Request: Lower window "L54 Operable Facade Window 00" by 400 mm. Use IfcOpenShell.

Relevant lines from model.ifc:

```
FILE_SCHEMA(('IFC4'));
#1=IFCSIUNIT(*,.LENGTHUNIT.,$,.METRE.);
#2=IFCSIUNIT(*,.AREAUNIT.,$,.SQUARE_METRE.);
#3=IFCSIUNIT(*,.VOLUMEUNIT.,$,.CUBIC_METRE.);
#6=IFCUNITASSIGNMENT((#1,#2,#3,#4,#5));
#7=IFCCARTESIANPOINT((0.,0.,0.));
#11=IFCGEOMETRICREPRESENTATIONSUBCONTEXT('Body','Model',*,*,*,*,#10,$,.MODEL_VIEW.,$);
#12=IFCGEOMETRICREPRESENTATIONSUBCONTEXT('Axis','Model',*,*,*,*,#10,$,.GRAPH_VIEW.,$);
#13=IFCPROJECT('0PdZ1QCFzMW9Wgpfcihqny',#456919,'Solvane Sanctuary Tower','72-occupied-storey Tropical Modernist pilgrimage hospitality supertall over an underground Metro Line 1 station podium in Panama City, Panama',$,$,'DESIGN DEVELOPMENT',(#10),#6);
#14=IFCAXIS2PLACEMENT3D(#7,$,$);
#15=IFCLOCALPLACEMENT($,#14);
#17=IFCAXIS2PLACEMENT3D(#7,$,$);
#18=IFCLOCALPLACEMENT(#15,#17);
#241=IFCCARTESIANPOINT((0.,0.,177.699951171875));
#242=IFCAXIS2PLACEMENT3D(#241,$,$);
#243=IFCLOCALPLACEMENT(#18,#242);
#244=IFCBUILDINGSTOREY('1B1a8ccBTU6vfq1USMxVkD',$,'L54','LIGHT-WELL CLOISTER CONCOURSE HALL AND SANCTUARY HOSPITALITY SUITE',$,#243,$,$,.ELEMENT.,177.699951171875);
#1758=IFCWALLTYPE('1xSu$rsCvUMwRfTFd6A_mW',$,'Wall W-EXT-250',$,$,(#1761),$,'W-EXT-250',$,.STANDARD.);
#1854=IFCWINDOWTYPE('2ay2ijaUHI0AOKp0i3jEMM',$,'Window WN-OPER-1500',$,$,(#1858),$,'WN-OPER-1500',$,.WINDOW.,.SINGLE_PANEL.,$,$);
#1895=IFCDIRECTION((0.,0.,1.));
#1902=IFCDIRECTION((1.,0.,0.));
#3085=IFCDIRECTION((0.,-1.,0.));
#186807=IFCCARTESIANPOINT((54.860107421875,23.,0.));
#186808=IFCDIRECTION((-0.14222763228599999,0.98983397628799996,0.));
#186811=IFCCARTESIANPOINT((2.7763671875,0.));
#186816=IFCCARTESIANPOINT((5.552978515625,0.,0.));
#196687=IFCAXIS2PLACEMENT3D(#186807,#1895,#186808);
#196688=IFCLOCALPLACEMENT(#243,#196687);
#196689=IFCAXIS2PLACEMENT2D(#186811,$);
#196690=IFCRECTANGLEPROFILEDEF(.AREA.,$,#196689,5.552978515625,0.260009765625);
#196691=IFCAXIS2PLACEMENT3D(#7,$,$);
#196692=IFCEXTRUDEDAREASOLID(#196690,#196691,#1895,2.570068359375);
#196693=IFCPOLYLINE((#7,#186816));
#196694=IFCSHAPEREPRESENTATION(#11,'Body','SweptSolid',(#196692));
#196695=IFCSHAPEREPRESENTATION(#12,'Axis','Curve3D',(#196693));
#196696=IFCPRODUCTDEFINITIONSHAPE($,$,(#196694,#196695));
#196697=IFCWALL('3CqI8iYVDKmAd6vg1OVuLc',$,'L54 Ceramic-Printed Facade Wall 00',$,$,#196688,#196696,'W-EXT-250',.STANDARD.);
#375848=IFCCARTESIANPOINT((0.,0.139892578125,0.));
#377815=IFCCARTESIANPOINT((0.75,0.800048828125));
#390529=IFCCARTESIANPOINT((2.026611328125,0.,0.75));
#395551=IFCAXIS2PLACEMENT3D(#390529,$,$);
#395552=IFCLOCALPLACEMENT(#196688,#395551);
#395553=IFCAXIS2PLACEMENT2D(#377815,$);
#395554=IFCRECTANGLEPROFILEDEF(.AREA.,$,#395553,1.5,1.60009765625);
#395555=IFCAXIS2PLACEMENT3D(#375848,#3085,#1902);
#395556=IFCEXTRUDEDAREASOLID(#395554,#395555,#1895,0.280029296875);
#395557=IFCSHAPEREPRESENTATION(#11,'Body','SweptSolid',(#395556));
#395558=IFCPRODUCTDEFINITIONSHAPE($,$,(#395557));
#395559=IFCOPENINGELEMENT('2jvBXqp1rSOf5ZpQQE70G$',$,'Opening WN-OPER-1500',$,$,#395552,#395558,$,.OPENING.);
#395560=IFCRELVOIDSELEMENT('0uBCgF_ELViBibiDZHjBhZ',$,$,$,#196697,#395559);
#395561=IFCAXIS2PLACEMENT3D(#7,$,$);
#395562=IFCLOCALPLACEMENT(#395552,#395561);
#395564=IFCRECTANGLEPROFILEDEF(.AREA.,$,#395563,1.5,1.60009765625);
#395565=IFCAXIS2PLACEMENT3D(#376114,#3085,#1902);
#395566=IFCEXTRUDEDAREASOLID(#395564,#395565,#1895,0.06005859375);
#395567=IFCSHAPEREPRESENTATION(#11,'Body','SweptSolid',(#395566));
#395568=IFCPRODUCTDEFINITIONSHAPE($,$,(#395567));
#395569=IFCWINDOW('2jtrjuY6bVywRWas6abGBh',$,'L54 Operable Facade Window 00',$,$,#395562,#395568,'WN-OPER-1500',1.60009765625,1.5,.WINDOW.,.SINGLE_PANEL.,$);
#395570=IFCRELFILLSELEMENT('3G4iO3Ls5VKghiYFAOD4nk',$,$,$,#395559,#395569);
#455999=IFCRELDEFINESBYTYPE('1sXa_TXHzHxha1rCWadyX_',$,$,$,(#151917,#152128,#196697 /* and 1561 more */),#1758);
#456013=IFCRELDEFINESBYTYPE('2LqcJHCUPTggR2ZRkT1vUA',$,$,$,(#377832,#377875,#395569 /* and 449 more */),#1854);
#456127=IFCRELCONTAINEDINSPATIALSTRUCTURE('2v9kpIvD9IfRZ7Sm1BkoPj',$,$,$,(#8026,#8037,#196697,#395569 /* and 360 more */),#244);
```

```python
import numpy as np
import ifcopenshell
import ifcopenshell.api.geometry
import ifcopenshell.util.placement
import ifcopenshell.util.unit

model = ifcopenshell.open("model.ifc")
unit_scale = ifcopenshell.util.unit.calculate_unit_scale(model)

window = model.by_guid("2jtrjuY6bVywRWas6abGBh")
opening = window.FillsVoids[0].RelatingOpeningElement
dz = -0.4 / unit_scale

shift = np.array([0.0, 0.0, dz])
# The window is placed relative to its opening, so it follows when the opening moves.
matrix = ifcopenshell.util.placement.get_local_placement(opening.ObjectPlacement)
matrix[:3, 3] += shift
ifcopenshell.api.geometry.edit_object_placement(
    model, product=opening, matrix=matrix, is_si=False, should_transform_children=True
)

print(f"moved by {dz * unit_scale:+.3f} m")

model.write("model_rev.ifc")
```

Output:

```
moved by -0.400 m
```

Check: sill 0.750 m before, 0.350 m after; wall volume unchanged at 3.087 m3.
